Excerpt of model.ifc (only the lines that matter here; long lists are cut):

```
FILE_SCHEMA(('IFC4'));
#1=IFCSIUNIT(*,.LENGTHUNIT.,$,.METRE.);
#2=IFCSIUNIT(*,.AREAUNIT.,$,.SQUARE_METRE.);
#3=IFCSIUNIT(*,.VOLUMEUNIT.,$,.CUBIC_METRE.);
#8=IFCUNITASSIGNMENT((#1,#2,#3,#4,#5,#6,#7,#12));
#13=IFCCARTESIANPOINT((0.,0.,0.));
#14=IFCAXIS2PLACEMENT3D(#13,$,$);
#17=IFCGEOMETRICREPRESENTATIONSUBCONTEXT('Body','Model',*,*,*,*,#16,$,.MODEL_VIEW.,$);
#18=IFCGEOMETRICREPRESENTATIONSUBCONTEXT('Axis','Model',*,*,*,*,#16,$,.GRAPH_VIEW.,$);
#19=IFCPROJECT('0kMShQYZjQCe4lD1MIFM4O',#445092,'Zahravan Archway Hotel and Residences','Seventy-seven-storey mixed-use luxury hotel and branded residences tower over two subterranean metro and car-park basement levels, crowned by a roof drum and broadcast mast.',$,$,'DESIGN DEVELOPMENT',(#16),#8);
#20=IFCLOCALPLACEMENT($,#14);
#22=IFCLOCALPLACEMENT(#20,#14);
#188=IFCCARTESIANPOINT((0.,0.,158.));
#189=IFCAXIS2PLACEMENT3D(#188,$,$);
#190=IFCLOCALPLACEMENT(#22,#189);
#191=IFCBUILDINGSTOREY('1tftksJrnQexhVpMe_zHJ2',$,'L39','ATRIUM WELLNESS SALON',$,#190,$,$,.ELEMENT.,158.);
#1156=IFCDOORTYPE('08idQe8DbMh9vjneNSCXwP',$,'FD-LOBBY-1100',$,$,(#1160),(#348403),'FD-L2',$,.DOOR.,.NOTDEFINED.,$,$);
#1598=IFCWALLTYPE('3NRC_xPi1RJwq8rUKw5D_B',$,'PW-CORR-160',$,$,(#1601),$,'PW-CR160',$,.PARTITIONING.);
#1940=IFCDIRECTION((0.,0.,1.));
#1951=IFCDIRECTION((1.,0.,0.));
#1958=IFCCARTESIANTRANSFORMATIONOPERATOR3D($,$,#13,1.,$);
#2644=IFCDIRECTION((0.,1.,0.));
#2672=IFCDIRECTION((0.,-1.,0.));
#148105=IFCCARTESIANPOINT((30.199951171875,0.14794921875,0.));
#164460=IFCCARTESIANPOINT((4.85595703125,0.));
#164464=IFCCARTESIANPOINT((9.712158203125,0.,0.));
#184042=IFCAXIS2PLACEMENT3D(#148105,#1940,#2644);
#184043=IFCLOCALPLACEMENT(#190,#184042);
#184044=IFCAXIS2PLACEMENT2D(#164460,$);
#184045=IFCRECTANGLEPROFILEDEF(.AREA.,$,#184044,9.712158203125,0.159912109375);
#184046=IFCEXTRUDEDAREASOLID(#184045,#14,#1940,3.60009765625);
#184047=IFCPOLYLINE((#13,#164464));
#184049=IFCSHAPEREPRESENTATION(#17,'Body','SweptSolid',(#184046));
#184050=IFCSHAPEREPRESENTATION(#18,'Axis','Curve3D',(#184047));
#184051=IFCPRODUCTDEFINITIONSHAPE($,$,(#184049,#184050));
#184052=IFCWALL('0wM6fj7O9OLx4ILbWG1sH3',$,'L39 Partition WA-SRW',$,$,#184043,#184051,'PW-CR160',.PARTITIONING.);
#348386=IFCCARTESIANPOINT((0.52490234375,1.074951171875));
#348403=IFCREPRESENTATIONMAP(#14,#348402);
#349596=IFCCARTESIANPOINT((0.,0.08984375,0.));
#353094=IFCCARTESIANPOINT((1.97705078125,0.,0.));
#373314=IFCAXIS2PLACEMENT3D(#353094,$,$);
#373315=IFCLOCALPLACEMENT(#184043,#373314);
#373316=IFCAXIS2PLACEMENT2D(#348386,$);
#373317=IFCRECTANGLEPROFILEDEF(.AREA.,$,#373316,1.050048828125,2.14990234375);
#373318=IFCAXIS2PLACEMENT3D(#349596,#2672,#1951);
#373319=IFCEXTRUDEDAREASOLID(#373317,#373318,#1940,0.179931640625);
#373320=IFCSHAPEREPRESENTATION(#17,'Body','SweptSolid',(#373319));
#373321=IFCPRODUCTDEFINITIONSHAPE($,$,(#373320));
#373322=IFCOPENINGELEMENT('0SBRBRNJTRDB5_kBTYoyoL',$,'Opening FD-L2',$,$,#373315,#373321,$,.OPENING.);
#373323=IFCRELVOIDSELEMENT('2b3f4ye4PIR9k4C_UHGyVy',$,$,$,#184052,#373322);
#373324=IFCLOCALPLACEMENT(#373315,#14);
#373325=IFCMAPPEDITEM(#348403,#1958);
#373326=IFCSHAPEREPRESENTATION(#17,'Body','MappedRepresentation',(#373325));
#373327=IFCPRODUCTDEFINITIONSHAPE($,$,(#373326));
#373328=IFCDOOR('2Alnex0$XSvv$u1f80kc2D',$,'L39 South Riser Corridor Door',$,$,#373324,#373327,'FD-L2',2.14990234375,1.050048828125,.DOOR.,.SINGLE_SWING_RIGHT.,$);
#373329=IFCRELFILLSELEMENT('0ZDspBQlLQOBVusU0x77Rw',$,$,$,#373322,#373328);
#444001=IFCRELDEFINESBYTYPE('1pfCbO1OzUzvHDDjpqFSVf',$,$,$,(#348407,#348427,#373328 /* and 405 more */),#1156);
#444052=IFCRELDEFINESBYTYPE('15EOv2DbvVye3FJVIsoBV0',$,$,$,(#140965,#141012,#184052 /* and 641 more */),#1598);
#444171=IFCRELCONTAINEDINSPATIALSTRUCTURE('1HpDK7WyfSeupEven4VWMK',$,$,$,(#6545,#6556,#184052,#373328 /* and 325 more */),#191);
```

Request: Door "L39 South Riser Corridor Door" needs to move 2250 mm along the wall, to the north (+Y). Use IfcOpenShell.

```python
import ifcopenshell
import ifcopenshell.api.geometry
import ifcopenshell.util.placement
import ifcopenshell.util.unit

model = ifcopenshell.open("model.ifc")
unit_scale = ifcopenshell.util.unit.calculate_unit_scale(model)

door = model.by_id(373328)
opening = door.FillsVoids[0].RelatingOpeningElement
wall = opening.VoidsElements[0].RelatingBuildingElement

wall_matrix = ifcopenshell.util.placement.get_local_placement(wall.ObjectPlacement)
shift = wall_matrix[:3, 0] * 2.25 / unit_scale
before = ifcopenshell.util.placement.get_local_placement(door.ObjectPlacement)[:3, 3].copy()

# The door is placed relative to its opening, so it follows when the opening moves.
matrix = ifcopenshell.util.placement.get_local_placement(opening.ObjectPlacement)
matrix[:3, 3] += shift
ifcopenshell.api.geometry.edit_object_placement(
    model, product=opening, matrix=matrix, is_si=False, should_transform_children=True
)

after = ifcopenshell.util.placement.get_local_placement(door.ObjectPlacement)[:3, 3]
print("door moved by", (after - before).round(3) + 0.0)

model.write("model_rev.ifc")
```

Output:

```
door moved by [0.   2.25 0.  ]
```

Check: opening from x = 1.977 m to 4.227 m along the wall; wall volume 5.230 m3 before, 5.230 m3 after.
